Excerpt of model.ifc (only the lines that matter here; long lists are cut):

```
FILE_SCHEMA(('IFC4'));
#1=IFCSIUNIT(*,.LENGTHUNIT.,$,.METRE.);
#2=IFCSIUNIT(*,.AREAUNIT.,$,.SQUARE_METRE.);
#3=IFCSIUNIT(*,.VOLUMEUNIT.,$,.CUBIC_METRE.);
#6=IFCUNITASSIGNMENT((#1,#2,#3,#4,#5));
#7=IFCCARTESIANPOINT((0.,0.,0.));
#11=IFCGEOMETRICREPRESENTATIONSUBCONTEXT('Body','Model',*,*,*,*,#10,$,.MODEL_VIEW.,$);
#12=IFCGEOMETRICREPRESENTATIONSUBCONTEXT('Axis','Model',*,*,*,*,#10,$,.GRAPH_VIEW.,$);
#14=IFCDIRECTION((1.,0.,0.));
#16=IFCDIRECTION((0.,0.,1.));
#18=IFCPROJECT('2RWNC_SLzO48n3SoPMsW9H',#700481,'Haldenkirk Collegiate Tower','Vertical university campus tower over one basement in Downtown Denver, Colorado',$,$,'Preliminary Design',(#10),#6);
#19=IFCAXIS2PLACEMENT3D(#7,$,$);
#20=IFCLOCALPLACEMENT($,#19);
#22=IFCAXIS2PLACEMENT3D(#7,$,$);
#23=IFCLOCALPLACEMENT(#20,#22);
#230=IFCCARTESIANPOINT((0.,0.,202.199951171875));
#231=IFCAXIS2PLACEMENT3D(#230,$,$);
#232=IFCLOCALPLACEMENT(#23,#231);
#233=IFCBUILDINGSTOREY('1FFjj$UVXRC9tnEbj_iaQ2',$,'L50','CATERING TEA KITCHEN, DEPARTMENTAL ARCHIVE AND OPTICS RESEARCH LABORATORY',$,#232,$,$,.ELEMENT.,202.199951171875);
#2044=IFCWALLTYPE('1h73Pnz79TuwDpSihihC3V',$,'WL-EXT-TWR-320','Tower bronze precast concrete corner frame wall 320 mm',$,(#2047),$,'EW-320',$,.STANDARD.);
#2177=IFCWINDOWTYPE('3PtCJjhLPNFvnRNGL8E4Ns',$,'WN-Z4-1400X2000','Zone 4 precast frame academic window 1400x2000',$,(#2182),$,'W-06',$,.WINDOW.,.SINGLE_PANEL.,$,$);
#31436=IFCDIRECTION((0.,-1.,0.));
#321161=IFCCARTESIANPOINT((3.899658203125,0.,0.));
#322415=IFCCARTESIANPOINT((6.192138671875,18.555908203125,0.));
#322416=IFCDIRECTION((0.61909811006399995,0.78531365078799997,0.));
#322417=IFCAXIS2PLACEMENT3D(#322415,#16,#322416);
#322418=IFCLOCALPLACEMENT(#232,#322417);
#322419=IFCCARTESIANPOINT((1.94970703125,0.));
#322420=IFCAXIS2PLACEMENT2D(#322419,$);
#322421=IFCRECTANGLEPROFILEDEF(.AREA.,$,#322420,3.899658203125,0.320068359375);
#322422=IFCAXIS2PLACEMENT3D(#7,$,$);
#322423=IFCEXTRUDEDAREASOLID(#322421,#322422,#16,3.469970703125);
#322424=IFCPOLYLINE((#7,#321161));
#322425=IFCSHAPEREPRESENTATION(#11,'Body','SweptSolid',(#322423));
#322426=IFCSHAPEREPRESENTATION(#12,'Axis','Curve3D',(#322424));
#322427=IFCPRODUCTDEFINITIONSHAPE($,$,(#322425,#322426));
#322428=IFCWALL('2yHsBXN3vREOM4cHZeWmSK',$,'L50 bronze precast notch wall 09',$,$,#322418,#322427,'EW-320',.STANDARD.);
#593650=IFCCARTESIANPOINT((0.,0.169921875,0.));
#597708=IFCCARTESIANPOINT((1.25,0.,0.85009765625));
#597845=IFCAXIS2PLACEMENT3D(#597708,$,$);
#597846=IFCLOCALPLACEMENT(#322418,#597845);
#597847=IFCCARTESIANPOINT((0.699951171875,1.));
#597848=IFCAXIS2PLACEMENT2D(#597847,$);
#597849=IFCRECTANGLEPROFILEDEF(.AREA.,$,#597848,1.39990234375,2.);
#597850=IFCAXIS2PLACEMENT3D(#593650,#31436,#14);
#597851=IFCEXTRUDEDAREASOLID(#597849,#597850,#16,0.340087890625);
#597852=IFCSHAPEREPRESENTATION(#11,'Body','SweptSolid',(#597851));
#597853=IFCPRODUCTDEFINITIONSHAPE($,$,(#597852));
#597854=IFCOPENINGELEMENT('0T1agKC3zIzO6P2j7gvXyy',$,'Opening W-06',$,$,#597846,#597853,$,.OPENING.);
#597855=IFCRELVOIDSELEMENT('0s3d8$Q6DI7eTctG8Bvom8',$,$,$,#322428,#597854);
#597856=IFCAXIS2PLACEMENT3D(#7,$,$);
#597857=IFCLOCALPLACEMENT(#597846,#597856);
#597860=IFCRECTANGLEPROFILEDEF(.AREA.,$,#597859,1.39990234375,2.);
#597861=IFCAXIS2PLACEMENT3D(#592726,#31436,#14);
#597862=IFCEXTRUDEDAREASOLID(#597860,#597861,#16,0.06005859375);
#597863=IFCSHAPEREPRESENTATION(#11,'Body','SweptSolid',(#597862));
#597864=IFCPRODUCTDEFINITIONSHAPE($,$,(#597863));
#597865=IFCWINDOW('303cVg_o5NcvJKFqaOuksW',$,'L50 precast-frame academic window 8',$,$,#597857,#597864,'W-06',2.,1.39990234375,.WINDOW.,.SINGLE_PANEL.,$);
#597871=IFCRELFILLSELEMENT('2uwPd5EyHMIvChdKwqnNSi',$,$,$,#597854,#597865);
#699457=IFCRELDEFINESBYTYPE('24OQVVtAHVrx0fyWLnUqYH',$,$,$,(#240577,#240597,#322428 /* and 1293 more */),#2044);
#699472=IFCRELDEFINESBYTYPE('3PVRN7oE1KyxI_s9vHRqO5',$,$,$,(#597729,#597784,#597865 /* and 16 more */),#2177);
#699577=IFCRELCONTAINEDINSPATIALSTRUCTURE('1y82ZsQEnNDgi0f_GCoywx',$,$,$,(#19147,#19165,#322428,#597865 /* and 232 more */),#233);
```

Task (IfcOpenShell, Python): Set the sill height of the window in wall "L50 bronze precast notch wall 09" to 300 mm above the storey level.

```python
import numpy as np
import ifcopenshell
import ifcopenshell.api.geometry
import ifcopenshell.geom
import ifcopenshell.util.element
import ifcopenshell.util.placement
import ifcopenshell.util.shape
import ifcopenshell.util.unit

model = ifcopenshell.open("model.ifc")
unit_scale = ifcopenshell.util.unit.calculate_unit_scale(model)

window = model.by_guid("303cVg_o5NcvJKFqaOuksW")
opening = window.FillsVoids[0].RelatingOpeningElement
storey = ifcopenshell.util.element.get_container(window, ifc_class="IfcBuildingStorey")
level = ifcopenshell.util.placement.get_local_placement(storey.ObjectPlacement)[2, 3]

# The opening's origin need not be at the sill, so measure its lowest point.
shape = ifcopenshell.geom.create_shape(ifcopenshell.geom.settings(), opening)
bottom = ifcopenshell.util.shape.get_shape_bottom_elevation(shape, shape.geometry) / unit_scale
dz = level + 0.3 / unit_scale - bottom

shift = np.array([0.0, 0.0, dz])
# The window is placed relative to its opening, so it follows when the opening moves.
matrix = ifcopenshell.util.placement.get_local_placement(opening.ObjectPlacement)
matrix[:3, 3] += shift
ifcopenshell.api.geometry.edit_object_placement(
    model, product=opening, matrix=matrix, is_si=False, should_transform_children=True
)

print(f"moved by {dz * unit_scale:+.3f} m")

model.write("model_v2.ifc")
```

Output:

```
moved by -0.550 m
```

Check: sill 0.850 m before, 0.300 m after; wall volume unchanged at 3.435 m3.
